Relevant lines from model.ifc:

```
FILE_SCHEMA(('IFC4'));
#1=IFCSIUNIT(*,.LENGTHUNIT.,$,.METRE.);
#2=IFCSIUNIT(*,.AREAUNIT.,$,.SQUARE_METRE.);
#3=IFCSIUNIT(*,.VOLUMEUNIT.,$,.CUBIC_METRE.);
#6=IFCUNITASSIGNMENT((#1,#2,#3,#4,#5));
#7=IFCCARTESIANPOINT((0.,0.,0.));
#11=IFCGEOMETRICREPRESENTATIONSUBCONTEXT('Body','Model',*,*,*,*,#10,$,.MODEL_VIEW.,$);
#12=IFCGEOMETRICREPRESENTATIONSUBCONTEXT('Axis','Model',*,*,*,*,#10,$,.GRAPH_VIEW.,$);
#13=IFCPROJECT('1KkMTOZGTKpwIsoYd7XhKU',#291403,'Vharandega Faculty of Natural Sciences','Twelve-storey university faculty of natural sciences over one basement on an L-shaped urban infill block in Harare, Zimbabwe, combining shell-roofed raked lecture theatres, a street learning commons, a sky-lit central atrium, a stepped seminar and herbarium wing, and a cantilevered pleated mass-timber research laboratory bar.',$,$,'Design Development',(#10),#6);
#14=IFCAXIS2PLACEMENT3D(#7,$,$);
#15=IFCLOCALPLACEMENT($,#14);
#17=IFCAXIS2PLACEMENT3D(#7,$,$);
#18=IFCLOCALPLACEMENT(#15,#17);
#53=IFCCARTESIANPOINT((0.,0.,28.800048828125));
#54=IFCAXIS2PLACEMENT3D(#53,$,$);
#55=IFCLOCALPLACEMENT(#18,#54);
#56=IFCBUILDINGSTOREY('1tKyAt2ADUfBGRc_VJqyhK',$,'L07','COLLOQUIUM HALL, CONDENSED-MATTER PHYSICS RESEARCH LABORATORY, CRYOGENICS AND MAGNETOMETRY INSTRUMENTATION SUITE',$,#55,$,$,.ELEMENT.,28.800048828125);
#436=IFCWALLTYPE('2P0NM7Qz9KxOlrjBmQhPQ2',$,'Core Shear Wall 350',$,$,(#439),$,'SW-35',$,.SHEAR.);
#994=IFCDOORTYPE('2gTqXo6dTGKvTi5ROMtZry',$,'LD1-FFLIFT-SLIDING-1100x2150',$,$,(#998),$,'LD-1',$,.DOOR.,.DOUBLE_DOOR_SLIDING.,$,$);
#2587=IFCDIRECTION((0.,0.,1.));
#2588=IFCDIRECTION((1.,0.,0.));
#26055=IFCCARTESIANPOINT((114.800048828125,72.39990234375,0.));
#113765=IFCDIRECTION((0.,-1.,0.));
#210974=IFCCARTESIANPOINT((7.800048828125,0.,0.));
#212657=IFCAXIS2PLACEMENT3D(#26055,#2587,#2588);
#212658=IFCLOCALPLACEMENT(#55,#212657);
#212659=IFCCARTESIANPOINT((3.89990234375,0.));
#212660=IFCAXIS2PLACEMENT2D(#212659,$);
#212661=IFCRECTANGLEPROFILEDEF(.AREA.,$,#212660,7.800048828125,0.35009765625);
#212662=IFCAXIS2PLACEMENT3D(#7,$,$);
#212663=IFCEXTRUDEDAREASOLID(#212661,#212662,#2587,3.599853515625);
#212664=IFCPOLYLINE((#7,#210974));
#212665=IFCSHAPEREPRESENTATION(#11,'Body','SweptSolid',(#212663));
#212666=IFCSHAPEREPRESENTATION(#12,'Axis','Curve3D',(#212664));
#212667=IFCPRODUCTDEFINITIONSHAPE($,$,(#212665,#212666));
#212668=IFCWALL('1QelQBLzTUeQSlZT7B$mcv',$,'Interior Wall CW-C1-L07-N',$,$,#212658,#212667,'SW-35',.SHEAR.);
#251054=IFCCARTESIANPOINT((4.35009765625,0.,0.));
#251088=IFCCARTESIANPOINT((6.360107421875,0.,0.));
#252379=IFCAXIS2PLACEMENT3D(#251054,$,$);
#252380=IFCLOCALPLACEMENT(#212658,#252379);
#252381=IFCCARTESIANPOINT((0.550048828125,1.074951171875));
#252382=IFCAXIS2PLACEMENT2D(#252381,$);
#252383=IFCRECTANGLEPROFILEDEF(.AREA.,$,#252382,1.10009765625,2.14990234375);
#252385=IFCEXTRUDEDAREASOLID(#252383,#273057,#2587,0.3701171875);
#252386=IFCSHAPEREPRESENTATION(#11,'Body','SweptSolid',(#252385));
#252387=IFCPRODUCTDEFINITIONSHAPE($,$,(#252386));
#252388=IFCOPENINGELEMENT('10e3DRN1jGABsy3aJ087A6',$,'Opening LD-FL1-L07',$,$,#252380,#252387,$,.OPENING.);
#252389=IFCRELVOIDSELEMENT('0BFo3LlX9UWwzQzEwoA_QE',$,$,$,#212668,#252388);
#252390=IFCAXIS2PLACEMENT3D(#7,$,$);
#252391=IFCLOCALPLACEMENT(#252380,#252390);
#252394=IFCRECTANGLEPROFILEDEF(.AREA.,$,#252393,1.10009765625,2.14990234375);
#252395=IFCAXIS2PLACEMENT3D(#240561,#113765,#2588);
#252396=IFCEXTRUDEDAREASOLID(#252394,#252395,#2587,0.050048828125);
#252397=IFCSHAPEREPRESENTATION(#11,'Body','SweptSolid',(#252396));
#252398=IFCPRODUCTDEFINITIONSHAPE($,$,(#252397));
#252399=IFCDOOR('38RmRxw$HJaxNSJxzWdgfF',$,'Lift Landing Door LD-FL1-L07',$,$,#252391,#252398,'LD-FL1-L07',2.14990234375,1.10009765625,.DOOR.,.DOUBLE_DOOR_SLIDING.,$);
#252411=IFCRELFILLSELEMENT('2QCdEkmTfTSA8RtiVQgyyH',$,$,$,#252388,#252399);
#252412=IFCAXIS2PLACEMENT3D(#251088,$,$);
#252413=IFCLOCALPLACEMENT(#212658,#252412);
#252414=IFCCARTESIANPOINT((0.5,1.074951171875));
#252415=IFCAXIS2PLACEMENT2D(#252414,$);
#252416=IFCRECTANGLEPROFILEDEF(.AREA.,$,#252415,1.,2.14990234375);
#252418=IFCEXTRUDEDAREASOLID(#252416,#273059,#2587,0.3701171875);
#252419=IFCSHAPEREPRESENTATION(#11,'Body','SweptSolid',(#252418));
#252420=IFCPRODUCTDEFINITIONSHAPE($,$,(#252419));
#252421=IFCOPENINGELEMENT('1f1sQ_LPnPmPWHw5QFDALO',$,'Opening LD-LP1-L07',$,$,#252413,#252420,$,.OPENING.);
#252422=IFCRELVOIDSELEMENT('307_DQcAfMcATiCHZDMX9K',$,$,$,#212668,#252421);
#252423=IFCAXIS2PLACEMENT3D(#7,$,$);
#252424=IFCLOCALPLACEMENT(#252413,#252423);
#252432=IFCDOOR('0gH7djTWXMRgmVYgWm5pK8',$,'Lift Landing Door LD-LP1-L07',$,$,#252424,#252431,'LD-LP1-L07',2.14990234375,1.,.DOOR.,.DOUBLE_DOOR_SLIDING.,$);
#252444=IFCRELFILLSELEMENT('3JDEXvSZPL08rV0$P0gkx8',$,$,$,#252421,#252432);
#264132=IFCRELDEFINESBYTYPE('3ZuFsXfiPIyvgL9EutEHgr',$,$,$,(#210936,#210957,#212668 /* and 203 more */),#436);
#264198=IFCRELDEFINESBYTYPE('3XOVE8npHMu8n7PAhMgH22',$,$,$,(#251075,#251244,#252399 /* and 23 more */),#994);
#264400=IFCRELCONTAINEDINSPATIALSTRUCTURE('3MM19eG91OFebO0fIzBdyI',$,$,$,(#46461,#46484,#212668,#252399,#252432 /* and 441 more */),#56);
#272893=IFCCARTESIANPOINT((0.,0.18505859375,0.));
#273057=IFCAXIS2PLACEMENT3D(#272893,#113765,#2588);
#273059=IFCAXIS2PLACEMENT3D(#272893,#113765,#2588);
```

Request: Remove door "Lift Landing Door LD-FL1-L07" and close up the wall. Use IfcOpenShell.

```python
import ifcopenshell
import ifcopenshell.api.feature
import ifcopenshell.api.root
import ifcopenshell.geom
import ifcopenshell.util.shape

model = ifcopenshell.open("model.ifc")
settings = ifcopenshell.geom.settings()


def volume(element):
    """Net volume in cubic metres, openings subtracted."""
    shape = ifcopenshell.geom.create_shape(settings, element)
    return ifcopenshell.util.shape.get_volume(shape.geometry)


door = model.by_guid("38RmRxw$HJaxNSJxzWdgfF")
opening = door.FillsVoids[0].RelatingOpeningElement
wall = opening.VoidsElements[0].RelatingBuildingElement
before = volume(wall)

ifcopenshell.api.root.remove_product(model, product=door)
ifcopenshell.api.feature.remove_feature(model, feature=opening)

after = volume(wall)

print(f"wall volume {before:.3f} -> {after:.3f} m3")

model.write("model_v2.ifc")
```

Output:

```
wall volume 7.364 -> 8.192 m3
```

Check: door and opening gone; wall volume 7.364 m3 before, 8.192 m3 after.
